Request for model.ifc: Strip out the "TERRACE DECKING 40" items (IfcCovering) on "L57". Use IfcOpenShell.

First a look at what the model holds.

```python
import ifcopenshell
import ifcopenshell.util.element

model = ifcopenshell.open("model.ifc")
print(model.schema)
storey = next(s for s in model.by_type("IfcBuildingStorey") if s.Name == "L57")
coverings = [e for e in ifcopenshell.util.element.get_decomposition(storey) if e.is_a("IfcCovering")]
seen = {}
for e in coverings:
    element_type = ifcopenshell.util.element.get_type(e)
    name = element_type.Name if element_type not in (None, e) else None
    seen[name] = seen.get(name, 0) + 1
for name, count in sorted(seen.items(), key=str):
    print(count, "x", name)
```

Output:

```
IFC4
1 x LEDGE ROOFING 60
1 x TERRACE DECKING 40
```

```python
import ifcopenshell
import ifcopenshell.api.root
import ifcopenshell.util.element

model = ifcopenshell.open("model.ifc")

storey = next(s for s in model.by_type("IfcBuildingStorey") if s.Name == "L57")
coverings = [e for e in ifcopenshell.util.element.get_decomposition(storey) if e.is_a("IfcCovering")]
targets = [e for e in coverings if (t := ifcopenshell.util.element.get_type(e)) not in (None, e) and t.Name == "TERRACE DECKING 40"]

for e in targets:
    ifcopenshell.api.root.remove_product(model, product=e)
print(len(targets), "removed")

model.write("model_updated.ifc")
```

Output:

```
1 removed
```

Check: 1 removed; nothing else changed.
